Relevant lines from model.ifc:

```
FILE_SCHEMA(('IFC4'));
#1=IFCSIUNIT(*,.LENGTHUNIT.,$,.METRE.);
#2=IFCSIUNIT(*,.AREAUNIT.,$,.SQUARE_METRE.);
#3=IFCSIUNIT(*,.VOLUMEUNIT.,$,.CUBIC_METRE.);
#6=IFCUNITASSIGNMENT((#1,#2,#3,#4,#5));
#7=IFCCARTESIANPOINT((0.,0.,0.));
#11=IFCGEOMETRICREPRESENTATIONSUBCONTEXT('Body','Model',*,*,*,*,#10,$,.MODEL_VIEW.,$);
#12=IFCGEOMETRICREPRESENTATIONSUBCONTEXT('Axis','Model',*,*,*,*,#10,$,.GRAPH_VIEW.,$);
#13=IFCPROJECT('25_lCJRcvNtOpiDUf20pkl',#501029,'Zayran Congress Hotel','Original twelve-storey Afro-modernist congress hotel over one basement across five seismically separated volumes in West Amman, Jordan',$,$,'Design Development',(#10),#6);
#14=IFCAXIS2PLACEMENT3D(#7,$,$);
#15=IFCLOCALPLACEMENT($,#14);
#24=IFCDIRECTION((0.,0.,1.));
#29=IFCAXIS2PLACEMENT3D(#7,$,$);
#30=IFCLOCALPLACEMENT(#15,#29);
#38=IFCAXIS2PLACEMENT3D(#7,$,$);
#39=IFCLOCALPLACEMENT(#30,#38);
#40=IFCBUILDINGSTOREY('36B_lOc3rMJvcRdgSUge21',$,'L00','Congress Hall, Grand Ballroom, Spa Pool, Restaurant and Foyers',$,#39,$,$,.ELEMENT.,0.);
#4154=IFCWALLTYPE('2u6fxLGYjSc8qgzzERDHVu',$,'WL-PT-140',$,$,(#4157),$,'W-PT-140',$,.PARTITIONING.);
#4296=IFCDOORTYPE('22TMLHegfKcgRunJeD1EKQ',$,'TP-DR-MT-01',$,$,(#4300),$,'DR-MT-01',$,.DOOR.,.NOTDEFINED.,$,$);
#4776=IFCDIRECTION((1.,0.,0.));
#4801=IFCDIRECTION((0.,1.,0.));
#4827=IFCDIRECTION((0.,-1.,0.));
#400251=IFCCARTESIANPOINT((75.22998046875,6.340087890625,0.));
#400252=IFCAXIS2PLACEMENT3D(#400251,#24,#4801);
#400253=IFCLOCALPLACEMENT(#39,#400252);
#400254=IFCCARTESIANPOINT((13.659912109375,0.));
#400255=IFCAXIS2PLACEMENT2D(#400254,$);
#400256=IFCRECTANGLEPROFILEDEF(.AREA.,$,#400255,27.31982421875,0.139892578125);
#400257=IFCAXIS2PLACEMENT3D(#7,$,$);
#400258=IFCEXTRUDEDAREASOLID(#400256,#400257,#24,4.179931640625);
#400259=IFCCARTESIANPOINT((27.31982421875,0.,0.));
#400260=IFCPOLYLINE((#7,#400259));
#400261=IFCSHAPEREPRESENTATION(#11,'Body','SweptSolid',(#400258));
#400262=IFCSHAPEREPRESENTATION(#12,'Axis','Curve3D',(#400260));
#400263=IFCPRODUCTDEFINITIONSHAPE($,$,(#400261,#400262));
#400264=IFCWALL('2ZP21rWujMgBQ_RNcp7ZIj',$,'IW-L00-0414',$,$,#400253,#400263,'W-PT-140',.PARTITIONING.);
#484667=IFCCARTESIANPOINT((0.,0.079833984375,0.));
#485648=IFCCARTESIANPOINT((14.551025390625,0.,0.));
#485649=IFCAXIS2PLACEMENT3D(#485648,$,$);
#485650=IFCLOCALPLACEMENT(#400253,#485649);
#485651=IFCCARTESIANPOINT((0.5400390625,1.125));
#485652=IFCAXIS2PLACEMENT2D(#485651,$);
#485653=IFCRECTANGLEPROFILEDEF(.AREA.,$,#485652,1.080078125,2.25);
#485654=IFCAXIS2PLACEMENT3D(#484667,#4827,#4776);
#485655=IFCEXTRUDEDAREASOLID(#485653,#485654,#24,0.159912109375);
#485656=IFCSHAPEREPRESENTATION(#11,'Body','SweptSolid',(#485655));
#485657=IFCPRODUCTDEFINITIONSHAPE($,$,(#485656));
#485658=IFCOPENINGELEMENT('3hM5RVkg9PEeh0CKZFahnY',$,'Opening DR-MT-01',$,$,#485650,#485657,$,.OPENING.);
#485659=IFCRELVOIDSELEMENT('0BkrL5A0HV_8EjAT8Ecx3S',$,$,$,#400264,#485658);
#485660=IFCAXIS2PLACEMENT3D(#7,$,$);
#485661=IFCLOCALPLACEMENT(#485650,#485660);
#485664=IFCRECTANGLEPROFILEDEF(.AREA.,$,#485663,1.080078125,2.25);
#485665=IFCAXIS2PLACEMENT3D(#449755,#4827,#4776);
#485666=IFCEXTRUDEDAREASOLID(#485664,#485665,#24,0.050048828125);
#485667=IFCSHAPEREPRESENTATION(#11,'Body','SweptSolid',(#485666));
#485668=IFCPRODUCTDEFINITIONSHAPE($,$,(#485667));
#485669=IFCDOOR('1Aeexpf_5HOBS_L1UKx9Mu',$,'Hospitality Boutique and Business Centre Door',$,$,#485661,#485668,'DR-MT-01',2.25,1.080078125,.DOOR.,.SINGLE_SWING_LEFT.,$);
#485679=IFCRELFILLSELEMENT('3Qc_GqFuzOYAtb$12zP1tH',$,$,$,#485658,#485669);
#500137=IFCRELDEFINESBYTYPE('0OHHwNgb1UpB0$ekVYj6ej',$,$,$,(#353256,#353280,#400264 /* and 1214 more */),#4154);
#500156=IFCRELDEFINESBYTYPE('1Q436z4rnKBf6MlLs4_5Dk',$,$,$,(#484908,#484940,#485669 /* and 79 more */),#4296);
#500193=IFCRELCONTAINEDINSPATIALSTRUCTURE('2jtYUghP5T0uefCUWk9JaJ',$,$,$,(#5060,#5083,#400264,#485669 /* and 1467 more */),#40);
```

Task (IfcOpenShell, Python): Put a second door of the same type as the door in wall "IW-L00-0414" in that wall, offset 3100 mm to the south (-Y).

```python
import ifcopenshell
import ifcopenshell.api.feature
import ifcopenshell.api.geometry
import ifcopenshell.api.root
import ifcopenshell.geom
import ifcopenshell.util.element
import ifcopenshell.util.placement
import ifcopenshell.util.shape
import ifcopenshell.util.unit

model = ifcopenshell.open("model.ifc")
unit_scale = ifcopenshell.util.unit.calculate_unit_scale(model)
settings = ifcopenshell.geom.settings()


def volume(element):
    """Net volume in cubic metres, openings subtracted."""
    shape = ifcopenshell.geom.create_shape(settings, element)
    return ifcopenshell.util.shape.get_volume(shape.geometry)


door = model.by_id(485669)
opening = door.FillsVoids[0].RelatingOpeningElement
wall = opening.VoidsElements[0].RelatingBuildingElement
before = volume(wall)
shift = ifcopenshell.util.placement.get_local_placement(wall.ObjectPlacement)[:3, 0] * -3.1 / unit_scale

# copy_class copies the void relationship, type, container and properties, but no geometry.
new_opening = ifcopenshell.api.root.copy_class(model, product=opening)
new_opening.Representation = ifcopenshell.util.element.copy_deep(
    model, opening.Representation, exclude=["IfcGeometricRepresentationContext", "IfcRepresentationMap"]
)
new_door = ifcopenshell.api.root.copy_class(model, product=door)
new_door.Representation = ifcopenshell.util.element.copy_deep(
    model, door.Representation, exclude=["IfcGeometricRepresentationContext", "IfcRepresentationMap"]
)
new_door.Tag = None
ifcopenshell.api.feature.add_filling(model, opening=new_opening, element=new_door)

for old, new in ((opening, new_opening), (door, new_door)):
    matrix = ifcopenshell.util.placement.get_local_placement(old.ObjectPlacement)
    matrix[:3, 3] += shift
    ifcopenshell.api.geometry.edit_object_placement(model, product=new, matrix=matrix, is_si=False)

after = volume(wall)

print(f"wall volume {before:.3f} -> {after:.3f} m3")

model.write("model-out.ifc")
```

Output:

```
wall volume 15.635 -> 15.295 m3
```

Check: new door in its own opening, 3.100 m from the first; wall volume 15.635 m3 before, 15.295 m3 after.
